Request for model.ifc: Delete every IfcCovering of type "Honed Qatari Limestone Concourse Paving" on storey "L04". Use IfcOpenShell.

First a look at what the model holds.

```python
import ifcopenshell
import ifcopenshell.util.element

model = ifcopenshell.open("model.ifc")
print(model.schema)
storey = next(s for s in model.by_type("IfcBuildingStorey") if s.Name == "L04")
coverings = [e for e in ifcopenshell.util.element.get_decomposition(storey) if e.is_a("IfcCovering")]
seen = {}
for e in coverings:
    element_type = ifcopenshell.util.element.get_type(e)
    name = element_type.Name if element_type not in (None, e) else None
    seen[name] = seen.get(name, 0) + 1
for name, count in sorted(seen.items(), key=str):
    print(count, "x", name)
```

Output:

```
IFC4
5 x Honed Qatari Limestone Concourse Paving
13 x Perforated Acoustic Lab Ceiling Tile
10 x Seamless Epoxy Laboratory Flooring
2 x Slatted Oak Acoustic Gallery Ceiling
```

```python
import ifcopenshell
import ifcopenshell.api.root
import ifcopenshell.util.element

model = ifcopenshell.open("model.ifc")

storey = next(s for s in model.by_type("IfcBuildingStorey") if s.Name == "L04")
coverings = [e for e in ifcopenshell.util.element.get_decomposition(storey) if e.is_a("IfcCovering")]
targets = [e for e in coverings if (t := ifcopenshell.util.element.get_type(e)) not in (None, e) and t.Name == "Honed Qatari Limestone Concourse Paving"]

for e in targets:
    ifcopenshell.api.root.remove_product(model, product=e)
print(len(targets), "removed")

model.write("model_rev.ifc")
```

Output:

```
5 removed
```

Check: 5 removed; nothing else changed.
